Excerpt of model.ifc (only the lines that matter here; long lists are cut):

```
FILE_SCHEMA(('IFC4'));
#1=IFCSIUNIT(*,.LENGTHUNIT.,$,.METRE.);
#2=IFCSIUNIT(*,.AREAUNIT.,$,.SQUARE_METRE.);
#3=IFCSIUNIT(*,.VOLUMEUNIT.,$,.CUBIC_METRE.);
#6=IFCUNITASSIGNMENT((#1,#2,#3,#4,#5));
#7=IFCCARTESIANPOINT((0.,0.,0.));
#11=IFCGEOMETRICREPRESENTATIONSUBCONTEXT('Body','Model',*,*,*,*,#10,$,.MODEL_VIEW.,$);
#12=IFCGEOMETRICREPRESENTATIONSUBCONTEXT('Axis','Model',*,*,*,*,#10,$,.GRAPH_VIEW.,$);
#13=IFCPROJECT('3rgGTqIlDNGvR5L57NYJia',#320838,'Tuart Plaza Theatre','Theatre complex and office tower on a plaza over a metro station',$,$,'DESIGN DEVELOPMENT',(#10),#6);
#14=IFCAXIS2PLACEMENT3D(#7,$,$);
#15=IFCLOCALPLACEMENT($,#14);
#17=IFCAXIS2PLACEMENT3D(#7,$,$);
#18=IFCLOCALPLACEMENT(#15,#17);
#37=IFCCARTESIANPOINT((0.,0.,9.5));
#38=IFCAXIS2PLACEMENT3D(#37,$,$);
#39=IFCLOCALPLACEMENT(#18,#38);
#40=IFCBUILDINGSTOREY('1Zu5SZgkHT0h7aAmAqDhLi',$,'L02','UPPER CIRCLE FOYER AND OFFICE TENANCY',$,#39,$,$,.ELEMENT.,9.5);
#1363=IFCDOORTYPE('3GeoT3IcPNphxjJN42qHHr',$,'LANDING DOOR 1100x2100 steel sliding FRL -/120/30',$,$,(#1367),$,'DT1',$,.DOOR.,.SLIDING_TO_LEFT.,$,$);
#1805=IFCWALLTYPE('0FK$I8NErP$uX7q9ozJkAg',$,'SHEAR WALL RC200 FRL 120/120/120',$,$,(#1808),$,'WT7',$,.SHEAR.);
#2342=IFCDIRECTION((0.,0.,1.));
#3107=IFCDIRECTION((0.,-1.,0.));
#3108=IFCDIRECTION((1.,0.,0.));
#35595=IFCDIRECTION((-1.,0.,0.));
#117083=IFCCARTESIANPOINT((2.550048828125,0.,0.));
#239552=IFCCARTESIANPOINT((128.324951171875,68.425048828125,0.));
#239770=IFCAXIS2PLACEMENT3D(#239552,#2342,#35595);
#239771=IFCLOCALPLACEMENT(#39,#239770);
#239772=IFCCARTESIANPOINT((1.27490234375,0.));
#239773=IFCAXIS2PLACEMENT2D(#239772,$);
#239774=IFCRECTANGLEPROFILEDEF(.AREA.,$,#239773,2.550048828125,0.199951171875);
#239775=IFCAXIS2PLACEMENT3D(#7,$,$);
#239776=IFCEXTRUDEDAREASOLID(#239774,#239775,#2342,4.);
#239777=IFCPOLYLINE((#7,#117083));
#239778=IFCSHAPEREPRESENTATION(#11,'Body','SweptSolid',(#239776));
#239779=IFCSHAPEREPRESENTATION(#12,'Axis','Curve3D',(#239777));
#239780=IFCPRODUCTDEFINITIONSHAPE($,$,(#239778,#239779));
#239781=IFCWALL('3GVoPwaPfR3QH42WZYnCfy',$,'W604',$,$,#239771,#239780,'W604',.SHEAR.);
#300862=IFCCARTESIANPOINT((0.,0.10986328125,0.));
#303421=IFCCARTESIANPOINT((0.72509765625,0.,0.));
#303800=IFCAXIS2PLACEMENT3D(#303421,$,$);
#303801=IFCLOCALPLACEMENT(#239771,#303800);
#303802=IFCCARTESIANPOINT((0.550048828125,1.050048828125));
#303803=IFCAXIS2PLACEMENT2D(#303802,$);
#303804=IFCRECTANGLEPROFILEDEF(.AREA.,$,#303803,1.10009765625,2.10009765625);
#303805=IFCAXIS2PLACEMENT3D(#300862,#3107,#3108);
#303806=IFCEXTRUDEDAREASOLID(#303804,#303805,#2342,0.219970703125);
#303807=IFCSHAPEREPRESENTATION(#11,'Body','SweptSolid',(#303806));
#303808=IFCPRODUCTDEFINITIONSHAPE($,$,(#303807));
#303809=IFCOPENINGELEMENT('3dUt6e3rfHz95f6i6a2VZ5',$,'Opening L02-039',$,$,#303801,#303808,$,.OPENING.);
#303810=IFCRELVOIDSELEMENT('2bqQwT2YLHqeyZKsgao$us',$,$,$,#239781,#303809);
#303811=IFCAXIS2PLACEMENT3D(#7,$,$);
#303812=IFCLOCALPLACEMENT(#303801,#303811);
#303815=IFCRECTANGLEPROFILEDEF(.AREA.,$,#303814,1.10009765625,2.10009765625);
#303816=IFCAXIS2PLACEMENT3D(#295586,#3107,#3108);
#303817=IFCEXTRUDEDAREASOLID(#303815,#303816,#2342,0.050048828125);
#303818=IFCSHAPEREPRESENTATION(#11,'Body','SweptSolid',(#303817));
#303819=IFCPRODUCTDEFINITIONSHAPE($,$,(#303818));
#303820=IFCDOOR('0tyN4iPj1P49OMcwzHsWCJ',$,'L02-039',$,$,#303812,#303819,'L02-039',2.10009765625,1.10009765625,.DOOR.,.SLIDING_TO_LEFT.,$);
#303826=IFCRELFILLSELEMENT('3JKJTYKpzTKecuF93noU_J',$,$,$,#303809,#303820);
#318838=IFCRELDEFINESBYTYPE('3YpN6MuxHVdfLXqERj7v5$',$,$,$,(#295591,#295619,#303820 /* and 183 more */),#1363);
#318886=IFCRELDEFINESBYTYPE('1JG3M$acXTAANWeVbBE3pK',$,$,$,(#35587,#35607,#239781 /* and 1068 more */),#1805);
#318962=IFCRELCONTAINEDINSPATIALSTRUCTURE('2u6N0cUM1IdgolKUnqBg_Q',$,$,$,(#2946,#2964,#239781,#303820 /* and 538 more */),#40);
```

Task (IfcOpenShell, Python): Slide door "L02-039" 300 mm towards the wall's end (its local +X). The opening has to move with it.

```python
import ifcopenshell
import ifcopenshell.api.geometry
import ifcopenshell.util.placement

model = ifcopenshell.open("model.ifc")

door = model.by_id(303820)
opening = door.FillsVoids[0].RelatingOpeningElement
wall = opening.VoidsElements[0].RelatingBuildingElement

wall_matrix = ifcopenshell.util.placement.get_local_placement(wall.ObjectPlacement)
shift = wall_matrix[:3, 0] * 0.3
before = ifcopenshell.util.placement.get_local_placement(door.ObjectPlacement)[:3, 3].copy()

# The door is placed relative to its opening, so it follows when the opening moves.
matrix = ifcopenshell.util.placement.get_local_placement(opening.ObjectPlacement)
matrix[:3, 3] += shift
ifcopenshell.api.geometry.edit_object_placement(
    model, product=opening, matrix=matrix, is_si=False, should_transform_children=True
)

after = ifcopenshell.util.placement.get_local_placement(door.ObjectPlacement)[:3, 3]
print("door moved by", (after - before).round(3) + 0.0)

model.write("model-out.ifc")
```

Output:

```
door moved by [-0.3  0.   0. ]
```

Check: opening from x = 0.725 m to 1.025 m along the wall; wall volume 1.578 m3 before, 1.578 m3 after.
